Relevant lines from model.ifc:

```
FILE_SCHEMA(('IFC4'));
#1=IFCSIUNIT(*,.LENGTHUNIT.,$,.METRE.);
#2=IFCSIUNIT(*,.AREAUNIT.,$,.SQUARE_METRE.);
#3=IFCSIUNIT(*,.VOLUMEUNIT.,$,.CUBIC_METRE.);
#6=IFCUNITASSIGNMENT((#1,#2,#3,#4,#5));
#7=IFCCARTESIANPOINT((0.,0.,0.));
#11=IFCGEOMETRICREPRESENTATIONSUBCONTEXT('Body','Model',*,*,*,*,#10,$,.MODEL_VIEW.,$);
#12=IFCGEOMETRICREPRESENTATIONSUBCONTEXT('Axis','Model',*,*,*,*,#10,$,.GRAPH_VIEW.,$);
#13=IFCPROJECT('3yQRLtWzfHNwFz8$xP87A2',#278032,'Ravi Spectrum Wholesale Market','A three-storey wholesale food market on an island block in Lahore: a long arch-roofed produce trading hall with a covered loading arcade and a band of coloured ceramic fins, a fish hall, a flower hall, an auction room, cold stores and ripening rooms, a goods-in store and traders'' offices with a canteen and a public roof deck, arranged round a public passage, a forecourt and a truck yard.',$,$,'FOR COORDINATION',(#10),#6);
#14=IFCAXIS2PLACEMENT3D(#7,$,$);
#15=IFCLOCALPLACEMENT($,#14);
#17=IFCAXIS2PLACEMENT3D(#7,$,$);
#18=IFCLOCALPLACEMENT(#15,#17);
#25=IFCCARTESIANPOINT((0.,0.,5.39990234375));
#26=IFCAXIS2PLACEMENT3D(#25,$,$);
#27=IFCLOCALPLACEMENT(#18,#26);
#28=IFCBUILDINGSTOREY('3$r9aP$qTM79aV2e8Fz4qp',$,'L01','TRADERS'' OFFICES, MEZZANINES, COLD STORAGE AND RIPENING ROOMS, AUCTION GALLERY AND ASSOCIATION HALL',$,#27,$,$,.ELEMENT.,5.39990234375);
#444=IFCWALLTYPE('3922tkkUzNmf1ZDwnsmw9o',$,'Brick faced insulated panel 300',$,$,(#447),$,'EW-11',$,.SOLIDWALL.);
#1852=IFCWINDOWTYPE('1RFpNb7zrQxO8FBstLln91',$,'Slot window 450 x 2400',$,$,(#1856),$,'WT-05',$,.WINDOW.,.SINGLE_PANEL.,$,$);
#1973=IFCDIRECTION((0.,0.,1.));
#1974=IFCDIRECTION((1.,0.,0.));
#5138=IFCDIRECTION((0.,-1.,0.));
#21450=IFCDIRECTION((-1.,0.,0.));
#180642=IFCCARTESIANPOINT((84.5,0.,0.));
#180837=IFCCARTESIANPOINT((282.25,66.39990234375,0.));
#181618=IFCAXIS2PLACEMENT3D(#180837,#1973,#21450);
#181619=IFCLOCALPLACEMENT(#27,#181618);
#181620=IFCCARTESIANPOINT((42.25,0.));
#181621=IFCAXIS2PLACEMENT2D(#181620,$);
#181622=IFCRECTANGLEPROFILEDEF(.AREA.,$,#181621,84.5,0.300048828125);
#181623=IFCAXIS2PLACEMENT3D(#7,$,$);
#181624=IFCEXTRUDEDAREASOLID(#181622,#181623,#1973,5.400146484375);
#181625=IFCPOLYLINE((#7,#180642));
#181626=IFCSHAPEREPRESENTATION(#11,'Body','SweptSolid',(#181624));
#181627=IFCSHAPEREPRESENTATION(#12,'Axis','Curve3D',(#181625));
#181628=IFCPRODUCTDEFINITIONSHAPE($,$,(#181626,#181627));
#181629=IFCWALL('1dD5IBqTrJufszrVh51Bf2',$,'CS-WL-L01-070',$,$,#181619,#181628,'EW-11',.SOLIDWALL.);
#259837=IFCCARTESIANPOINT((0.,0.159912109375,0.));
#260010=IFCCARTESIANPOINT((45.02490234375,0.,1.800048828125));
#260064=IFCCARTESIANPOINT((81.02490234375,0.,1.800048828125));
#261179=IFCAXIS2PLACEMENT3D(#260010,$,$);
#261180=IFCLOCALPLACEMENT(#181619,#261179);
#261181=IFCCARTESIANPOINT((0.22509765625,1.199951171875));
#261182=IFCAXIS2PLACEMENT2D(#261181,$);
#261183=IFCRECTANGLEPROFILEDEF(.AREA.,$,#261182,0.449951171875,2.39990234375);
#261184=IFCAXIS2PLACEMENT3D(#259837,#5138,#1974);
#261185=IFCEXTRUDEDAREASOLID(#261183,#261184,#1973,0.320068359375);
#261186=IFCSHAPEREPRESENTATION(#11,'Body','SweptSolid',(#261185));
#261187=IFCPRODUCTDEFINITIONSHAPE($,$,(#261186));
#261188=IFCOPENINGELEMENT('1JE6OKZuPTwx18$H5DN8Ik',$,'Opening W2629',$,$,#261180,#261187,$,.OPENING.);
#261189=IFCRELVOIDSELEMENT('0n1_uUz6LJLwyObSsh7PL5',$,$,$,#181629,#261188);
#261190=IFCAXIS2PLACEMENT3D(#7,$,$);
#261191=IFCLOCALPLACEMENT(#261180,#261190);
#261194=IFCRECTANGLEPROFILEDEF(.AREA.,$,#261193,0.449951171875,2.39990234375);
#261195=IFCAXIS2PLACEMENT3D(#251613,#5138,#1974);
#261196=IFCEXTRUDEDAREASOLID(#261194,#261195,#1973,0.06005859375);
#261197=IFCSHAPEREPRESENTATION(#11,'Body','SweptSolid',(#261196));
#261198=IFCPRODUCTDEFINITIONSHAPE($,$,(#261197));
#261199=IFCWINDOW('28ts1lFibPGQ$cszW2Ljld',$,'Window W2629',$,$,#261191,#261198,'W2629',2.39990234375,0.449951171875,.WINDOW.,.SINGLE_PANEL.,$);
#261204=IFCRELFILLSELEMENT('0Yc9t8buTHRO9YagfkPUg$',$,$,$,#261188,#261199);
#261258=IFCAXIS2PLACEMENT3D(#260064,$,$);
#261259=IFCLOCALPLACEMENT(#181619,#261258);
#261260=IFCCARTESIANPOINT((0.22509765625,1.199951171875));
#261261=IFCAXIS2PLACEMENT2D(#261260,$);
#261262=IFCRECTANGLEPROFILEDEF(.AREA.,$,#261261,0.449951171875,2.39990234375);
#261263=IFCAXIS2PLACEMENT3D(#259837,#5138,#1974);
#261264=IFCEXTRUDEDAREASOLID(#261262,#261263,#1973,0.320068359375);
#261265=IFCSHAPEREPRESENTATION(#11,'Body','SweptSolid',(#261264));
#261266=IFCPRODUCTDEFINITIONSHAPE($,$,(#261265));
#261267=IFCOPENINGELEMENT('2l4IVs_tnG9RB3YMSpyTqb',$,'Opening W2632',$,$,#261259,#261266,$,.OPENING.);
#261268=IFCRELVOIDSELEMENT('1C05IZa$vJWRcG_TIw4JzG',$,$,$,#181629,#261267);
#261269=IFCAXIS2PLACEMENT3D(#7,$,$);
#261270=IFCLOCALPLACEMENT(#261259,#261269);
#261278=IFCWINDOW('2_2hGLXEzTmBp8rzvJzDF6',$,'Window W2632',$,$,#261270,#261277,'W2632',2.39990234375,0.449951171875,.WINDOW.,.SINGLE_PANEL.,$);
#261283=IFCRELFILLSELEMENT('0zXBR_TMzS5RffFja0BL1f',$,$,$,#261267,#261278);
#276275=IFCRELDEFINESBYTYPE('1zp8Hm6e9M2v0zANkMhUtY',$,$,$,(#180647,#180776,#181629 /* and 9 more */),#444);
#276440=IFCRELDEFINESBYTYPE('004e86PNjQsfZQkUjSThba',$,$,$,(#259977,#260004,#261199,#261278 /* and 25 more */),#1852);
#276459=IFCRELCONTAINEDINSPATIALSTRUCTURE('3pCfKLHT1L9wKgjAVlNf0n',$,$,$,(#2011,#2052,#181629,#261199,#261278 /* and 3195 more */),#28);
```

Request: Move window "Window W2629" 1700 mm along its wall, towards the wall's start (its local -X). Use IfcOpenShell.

```python
import ifcopenshell
import ifcopenshell.api.geometry
import ifcopenshell.util.placement

model = ifcopenshell.open("model.ifc")

window = model.by_guid("28ts1lFibPGQ$cszW2Ljld")
opening = window.FillsVoids[0].RelatingOpeningElement
wall = opening.VoidsElements[0].RelatingBuildingElement

wall_matrix = ifcopenshell.util.placement.get_local_placement(wall.ObjectPlacement)
shift = wall_matrix[:3, 0] * -1.7
before = ifcopenshell.util.placement.get_local_placement(window.ObjectPlacement)[:3, 3].copy()

# The window is placed relative to its opening, so it follows when the opening moves.
matrix = ifcopenshell.util.placement.get_local_placement(opening.ObjectPlacement)
matrix[:3, 3] += shift
ifcopenshell.api.geometry.edit_object_placement(
    model, product=opening, matrix=matrix, is_si=False, should_transform_children=True
)

after = ifcopenshell.util.placement.get_local_placement(window.ObjectPlacement)[:3, 3]
print("window moved by", (after - before).round(3) + 0.0)

model.write("model_updated.ifc")
```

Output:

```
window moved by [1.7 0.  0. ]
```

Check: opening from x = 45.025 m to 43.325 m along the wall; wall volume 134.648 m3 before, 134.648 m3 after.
